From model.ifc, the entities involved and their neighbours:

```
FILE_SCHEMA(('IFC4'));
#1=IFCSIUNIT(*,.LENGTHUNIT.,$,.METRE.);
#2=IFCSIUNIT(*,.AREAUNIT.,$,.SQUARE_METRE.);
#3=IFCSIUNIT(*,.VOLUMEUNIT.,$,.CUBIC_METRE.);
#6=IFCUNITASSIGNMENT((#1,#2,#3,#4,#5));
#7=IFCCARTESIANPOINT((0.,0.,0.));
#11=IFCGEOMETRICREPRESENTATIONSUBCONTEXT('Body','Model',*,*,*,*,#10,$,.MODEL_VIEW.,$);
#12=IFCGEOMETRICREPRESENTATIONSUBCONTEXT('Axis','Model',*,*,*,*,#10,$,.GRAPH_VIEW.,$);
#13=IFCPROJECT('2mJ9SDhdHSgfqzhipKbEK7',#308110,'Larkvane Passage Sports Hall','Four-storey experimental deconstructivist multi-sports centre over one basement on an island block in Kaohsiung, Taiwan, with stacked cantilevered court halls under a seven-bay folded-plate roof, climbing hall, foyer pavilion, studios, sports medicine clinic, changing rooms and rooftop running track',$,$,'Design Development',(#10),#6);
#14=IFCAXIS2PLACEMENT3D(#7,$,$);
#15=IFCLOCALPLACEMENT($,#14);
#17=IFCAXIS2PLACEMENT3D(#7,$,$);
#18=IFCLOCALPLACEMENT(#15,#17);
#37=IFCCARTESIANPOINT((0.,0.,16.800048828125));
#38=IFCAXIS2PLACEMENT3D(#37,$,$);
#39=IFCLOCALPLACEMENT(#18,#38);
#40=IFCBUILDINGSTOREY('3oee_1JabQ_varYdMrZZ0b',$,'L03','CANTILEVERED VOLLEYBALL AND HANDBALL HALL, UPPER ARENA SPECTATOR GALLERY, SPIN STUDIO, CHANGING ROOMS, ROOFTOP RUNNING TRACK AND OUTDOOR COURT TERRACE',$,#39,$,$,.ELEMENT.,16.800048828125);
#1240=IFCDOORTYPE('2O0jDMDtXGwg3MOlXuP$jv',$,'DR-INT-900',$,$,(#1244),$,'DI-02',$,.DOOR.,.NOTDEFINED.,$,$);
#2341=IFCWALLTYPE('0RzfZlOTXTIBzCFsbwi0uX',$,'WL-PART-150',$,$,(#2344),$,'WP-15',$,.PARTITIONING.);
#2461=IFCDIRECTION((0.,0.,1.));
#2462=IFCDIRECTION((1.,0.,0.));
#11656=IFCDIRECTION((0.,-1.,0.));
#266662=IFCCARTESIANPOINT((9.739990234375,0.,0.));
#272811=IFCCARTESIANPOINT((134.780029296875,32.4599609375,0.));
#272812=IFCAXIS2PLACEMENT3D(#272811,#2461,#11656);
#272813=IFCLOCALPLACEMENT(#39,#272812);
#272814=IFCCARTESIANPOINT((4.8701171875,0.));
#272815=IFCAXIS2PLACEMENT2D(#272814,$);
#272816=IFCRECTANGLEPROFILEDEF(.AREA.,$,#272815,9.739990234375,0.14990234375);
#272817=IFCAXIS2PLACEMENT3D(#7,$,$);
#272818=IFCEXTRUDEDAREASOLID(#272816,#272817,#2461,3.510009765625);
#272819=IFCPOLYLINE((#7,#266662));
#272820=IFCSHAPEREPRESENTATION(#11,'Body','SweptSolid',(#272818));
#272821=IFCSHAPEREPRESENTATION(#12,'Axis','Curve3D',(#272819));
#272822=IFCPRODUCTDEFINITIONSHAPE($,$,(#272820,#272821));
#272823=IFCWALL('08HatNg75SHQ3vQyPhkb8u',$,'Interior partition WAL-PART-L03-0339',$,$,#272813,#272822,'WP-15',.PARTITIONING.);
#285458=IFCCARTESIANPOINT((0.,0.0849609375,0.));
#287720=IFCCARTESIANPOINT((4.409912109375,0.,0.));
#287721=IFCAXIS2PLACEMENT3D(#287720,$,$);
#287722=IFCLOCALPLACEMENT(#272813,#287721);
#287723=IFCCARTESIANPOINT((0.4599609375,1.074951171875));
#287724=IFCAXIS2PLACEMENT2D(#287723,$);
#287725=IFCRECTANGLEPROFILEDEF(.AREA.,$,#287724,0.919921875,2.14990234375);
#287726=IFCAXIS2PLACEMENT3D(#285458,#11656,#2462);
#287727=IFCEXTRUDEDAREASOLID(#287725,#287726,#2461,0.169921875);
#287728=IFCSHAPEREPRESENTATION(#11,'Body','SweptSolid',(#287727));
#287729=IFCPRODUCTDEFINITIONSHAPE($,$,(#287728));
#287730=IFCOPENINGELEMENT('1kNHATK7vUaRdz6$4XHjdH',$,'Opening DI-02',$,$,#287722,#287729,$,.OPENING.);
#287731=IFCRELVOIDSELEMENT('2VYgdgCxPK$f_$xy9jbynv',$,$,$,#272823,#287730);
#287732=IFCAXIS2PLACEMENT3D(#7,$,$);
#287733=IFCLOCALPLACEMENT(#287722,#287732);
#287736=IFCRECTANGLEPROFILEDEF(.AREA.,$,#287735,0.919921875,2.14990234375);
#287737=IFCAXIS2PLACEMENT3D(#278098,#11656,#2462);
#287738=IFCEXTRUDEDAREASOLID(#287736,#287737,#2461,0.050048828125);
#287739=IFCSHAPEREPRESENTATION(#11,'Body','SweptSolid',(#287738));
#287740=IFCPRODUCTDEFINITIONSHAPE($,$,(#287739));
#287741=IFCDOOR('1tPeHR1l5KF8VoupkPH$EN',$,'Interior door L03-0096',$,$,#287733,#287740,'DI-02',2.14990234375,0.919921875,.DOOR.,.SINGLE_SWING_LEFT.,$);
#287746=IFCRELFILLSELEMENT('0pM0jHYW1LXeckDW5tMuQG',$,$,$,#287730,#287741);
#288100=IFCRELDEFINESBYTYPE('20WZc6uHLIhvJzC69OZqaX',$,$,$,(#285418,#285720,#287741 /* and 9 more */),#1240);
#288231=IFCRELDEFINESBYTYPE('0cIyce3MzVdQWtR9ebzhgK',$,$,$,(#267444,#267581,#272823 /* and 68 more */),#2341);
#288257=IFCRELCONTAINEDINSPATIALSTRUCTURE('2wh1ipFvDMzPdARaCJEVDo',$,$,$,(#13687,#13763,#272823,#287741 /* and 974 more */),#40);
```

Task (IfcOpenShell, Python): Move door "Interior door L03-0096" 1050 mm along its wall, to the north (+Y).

```python
import ifcopenshell
import ifcopenshell.api.geometry
import ifcopenshell.util.placement

model = ifcopenshell.open("model.ifc")

door = model.by_guid("1tPeHR1l5KF8VoupkPH$EN")
opening = door.FillsVoids[0].RelatingOpeningElement
wall = opening.VoidsElements[0].RelatingBuildingElement

wall_matrix = ifcopenshell.util.placement.get_local_placement(wall.ObjectPlacement)
shift = wall_matrix[:3, 0] * -1.05
before = ifcopenshell.util.placement.get_local_placement(door.ObjectPlacement)[:3, 3].copy()

# The door is placed relative to its opening, so it follows when the opening moves.
matrix = ifcopenshell.util.placement.get_local_placement(opening.ObjectPlacement)
matrix[:3, 3] += shift
ifcopenshell.api.geometry.edit_object_placement(
    model, product=opening, matrix=matrix, is_si=False, should_transform_children=True
)

after = ifcopenshell.util.placement.get_local_placement(door.ObjectPlacement)[:3, 3]
print("door moved by", (after - before).round(3) + 0.0)

model.write("model_updated.ifc")
```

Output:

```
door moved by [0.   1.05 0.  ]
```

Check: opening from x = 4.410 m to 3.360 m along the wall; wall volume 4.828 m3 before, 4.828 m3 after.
